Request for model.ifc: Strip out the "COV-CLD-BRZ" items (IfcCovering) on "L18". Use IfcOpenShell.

First a look at what the model holds.

```python
import ifcopenshell
import ifcopenshell.util.element

model = ifcopenshell.open("model.ifc")
print(model.schema)
storey = next(s for s in model.by_type("IfcBuildingStorey") if s.Name == "L18")
coverings = [e for e in ifcopenshell.util.element.get_decomposition(storey) if e.is_a("IfcCovering")]
seen = {}
for e in coverings:
    element_type = ifcopenshell.util.element.get_type(e)
    name = element_type.Name if element_type not in (None, e) else None
    seen[name] = seen.get(name, 0) + 1
for name, count in sorted(seen.items(), key=str):
    print(count, "x", name)
```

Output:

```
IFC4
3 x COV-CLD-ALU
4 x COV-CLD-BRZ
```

```python
import ifcopenshell
import ifcopenshell.api.root
import ifcopenshell.util.element

model = ifcopenshell.open("model.ifc")

storey = next(s for s in model.by_type("IfcBuildingStorey") if s.Name == "L18")
coverings = [e for e in ifcopenshell.util.element.get_decomposition(storey) if e.is_a("IfcCovering")]
targets = [e for e in coverings if (t := ifcopenshell.util.element.get_type(e)) not in (None, e) and t.Name == "COV-CLD-BRZ"]

for e in targets:
    ifcopenshell.api.root.remove_product(model, product=e)
print(len(targets), "removed")

model.write("model-out.ifc")
```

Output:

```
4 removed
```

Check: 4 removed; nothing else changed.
